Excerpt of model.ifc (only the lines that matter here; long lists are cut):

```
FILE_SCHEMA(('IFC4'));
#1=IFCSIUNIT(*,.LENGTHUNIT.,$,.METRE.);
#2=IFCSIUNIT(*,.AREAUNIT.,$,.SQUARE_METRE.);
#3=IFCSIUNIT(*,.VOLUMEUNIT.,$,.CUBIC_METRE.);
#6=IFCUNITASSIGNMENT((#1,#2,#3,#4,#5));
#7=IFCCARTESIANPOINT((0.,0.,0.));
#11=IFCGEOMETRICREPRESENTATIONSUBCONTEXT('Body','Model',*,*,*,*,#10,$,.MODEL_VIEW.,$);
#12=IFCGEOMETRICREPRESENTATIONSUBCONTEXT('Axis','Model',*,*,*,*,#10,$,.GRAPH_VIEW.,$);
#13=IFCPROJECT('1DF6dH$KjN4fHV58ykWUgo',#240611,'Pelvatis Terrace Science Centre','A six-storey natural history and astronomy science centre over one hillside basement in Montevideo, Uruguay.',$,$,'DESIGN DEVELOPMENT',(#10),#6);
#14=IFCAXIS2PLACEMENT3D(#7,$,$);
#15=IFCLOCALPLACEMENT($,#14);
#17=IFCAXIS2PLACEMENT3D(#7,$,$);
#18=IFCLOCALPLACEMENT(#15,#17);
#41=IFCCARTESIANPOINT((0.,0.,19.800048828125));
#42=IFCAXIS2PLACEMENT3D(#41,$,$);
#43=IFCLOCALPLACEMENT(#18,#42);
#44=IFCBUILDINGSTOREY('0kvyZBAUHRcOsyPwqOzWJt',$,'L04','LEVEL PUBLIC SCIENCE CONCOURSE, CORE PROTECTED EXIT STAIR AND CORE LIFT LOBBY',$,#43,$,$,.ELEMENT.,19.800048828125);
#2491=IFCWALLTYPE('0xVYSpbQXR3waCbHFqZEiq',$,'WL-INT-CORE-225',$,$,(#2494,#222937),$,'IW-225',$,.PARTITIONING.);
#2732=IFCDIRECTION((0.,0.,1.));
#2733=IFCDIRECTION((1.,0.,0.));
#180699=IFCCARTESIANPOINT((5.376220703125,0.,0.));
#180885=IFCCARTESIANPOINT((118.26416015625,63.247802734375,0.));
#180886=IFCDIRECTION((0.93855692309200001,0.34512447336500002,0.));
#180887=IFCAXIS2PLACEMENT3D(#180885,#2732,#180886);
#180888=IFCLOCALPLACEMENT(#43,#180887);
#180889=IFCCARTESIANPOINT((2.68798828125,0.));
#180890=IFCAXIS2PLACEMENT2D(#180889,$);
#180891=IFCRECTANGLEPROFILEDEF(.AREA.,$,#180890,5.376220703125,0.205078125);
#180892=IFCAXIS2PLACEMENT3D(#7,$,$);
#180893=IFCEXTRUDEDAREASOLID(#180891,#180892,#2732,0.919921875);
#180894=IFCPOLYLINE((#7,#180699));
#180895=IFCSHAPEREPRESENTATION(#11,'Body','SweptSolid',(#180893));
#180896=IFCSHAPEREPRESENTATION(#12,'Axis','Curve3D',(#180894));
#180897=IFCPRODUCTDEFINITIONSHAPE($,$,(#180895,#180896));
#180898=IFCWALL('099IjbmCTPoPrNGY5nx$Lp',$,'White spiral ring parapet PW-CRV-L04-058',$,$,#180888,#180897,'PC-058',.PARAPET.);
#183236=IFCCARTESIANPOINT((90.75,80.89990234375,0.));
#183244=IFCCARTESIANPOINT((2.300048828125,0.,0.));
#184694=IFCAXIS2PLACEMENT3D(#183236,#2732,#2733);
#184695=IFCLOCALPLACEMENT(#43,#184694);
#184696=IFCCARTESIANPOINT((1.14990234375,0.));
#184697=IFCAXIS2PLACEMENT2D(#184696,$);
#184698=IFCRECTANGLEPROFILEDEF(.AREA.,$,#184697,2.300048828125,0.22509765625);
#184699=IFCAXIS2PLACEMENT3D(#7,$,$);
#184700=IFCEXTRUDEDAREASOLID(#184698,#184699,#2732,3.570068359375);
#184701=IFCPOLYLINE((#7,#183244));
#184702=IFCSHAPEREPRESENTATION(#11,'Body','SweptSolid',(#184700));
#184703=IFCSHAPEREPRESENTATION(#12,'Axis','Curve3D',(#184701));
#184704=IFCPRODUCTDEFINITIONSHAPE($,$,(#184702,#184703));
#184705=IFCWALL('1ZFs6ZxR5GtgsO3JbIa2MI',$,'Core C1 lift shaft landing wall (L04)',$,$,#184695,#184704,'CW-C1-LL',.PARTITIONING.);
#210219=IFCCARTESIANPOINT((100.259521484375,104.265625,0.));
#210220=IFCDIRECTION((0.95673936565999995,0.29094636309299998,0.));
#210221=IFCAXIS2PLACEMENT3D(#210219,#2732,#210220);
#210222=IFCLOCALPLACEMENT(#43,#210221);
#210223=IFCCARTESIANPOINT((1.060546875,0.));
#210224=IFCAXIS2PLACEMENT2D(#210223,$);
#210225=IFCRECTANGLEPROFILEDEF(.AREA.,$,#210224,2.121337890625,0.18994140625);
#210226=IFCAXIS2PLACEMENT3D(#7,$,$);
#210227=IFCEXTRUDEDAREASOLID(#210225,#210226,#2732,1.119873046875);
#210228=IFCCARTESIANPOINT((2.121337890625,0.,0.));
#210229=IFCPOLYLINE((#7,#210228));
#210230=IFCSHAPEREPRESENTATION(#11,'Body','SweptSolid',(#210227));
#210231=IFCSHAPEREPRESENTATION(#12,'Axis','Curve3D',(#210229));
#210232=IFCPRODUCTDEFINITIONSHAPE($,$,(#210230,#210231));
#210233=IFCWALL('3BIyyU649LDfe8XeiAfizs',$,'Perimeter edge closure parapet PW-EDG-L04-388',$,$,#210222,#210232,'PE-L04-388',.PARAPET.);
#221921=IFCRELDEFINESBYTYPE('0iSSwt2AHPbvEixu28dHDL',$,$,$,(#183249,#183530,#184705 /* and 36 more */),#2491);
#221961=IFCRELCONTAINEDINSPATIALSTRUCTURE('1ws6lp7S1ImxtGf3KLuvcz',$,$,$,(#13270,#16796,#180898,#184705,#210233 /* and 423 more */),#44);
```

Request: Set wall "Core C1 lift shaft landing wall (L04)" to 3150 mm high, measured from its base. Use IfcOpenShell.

```python
import ifcopenshell
import ifcopenshell.geom
import ifcopenshell.util.representation
import ifcopenshell.util.shape
import ifcopenshell.util.unit

model = ifcopenshell.open("model.ifc")
unit_scale = ifcopenshell.util.unit.calculate_unit_scale(model)
settings = ifcopenshell.geom.settings()


def volume(element):
    """Net volume in cubic metres, openings subtracted."""
    shape = ifcopenshell.geom.create_shape(settings, element)
    return ifcopenshell.util.shape.get_volume(shape.geometry)


wall = model.by_guid("1ZFs6ZxR5GtgsO3JbIa2MI")
before = volume(wall)

body = ifcopenshell.util.representation.get_representation(wall, "Model", "Body")
solid = body.Items[0]
old_height = solid.Depth
solid.Depth = 3.15 / unit_scale
after = volume(wall)

print(f"height {old_height:g} -> {solid.Depth:g}, volume {before:.3f} -> {after:.3f} m3")

model.write("model_rev.ifc")
```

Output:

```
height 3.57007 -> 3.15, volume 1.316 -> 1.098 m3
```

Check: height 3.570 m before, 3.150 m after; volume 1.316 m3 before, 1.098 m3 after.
